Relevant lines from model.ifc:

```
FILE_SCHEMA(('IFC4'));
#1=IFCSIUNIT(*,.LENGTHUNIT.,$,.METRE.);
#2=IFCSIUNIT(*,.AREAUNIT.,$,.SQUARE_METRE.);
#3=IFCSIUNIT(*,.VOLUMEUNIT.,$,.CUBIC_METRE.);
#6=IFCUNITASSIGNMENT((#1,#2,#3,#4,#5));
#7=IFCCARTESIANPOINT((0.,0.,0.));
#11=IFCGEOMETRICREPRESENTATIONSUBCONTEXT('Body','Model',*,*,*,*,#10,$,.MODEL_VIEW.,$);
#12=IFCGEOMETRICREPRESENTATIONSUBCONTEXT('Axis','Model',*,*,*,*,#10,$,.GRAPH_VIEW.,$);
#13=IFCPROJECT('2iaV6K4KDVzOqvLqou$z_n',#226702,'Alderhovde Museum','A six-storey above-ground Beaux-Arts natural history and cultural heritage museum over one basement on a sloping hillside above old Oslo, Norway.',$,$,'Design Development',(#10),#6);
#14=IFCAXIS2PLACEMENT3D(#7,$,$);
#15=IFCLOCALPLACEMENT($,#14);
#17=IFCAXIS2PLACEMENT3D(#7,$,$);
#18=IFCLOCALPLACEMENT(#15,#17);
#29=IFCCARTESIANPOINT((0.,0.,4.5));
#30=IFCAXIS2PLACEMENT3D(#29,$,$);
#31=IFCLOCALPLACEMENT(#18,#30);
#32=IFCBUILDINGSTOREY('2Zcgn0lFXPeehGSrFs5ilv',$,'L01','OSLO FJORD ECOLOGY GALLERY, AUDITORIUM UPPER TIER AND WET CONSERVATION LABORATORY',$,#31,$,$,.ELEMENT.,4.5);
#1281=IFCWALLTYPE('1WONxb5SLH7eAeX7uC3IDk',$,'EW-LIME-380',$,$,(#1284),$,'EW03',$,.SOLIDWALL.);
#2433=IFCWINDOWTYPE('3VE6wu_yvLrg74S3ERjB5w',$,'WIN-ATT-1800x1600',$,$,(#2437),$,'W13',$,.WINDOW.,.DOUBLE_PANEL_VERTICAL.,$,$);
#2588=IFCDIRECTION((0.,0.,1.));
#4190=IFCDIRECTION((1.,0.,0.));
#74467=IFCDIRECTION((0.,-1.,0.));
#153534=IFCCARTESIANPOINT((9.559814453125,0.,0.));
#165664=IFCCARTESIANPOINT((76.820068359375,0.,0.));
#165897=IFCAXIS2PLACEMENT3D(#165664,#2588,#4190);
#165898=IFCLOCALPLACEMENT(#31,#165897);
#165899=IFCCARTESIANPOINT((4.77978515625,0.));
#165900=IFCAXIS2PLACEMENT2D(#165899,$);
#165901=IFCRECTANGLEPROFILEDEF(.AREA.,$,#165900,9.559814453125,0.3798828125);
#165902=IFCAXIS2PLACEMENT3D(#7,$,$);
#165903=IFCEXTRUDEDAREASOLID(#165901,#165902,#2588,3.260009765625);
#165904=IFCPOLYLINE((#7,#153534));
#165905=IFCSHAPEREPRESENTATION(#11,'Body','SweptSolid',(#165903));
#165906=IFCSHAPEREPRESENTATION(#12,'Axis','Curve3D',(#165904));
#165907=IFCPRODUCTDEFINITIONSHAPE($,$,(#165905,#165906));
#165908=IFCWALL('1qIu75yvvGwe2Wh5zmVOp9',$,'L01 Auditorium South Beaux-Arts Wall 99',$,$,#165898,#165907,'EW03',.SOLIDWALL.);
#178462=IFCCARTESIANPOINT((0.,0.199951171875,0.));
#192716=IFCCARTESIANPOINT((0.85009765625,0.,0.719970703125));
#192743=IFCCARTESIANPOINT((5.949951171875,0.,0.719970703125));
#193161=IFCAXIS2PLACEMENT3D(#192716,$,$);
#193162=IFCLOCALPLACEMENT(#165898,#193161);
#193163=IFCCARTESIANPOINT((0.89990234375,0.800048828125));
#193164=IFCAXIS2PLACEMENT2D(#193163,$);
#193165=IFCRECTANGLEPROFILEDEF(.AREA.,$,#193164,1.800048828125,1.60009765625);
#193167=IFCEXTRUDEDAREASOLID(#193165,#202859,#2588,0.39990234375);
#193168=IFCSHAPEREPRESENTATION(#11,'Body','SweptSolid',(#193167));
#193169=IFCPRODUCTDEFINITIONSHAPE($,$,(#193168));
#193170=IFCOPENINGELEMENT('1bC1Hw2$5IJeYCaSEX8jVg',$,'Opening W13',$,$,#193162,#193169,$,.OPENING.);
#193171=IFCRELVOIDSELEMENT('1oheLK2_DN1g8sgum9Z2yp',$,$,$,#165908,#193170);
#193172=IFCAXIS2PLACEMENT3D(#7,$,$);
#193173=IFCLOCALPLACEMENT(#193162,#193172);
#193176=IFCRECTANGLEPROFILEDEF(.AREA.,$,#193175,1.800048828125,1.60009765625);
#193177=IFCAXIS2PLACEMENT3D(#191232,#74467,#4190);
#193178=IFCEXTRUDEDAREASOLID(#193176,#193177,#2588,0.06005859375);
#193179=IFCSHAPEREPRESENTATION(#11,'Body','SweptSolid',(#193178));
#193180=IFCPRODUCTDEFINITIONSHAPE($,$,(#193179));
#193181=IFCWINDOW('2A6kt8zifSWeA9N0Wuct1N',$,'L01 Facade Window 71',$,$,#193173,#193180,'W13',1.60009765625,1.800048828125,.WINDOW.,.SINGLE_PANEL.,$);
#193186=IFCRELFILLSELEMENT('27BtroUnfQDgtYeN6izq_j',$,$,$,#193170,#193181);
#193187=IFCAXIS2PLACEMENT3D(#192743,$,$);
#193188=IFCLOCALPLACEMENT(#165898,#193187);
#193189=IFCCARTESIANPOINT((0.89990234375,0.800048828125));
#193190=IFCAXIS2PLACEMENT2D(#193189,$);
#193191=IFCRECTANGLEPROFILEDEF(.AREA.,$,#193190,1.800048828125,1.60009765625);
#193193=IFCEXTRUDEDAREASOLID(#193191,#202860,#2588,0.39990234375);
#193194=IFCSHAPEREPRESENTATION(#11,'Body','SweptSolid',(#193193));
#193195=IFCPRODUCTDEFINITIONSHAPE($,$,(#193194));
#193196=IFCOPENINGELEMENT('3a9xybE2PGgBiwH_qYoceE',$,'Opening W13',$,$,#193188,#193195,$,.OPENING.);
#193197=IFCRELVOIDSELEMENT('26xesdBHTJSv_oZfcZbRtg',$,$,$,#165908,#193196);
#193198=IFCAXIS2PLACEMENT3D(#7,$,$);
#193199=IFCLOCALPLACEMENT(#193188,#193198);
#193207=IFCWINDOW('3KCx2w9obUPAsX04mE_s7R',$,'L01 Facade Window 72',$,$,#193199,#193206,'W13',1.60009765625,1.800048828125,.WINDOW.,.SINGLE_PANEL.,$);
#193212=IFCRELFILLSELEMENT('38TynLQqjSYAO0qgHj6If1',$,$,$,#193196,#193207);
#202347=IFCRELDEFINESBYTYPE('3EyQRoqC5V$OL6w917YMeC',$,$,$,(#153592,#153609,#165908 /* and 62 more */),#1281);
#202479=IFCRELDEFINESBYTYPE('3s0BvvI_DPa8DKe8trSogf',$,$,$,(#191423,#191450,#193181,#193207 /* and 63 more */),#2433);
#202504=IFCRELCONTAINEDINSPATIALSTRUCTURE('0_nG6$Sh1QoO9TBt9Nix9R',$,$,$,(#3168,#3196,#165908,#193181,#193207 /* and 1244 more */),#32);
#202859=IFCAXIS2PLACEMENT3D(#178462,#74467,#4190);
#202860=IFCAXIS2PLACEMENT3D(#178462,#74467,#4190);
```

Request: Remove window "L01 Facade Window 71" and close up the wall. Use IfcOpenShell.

```python
import ifcopenshell
import ifcopenshell.api.feature
import ifcopenshell.api.root
import ifcopenshell.geom
import ifcopenshell.util.shape

model = ifcopenshell.open("model.ifc")
settings = ifcopenshell.geom.settings()


def volume(element):
    """Net volume in cubic metres, openings subtracted."""
    shape = ifcopenshell.geom.create_shape(settings, element)
    return ifcopenshell.util.shape.get_volume(shape.geometry)


window = model.by_guid("2A6kt8zifSWeA9N0Wuct1N")
opening = window.FillsVoids[0].RelatingOpeningElement
wall = opening.VoidsElements[0].RelatingBuildingElement
before = volume(wall)

ifcopenshell.api.root.remove_product(model, product=window)
ifcopenshell.api.feature.remove_feature(model, feature=opening)

after = volume(wall)

print(f"wall volume {before:.3f} -> {after:.3f} m3")

model.write("model_v2.ifc")
```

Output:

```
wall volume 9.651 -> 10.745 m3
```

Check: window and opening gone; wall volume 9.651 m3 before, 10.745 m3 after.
